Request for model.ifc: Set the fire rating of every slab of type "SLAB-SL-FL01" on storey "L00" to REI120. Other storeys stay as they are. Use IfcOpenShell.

First a look at what the model holds.

```python
import ifcopenshell
import ifcopenshell.util.element

model = ifcopenshell.open("model.ifc")
print(model.schema)
storey = next(s for s in model.by_type("IfcBuildingStorey") if s.Name == "L00")
slabs = [e for e in ifcopenshell.util.element.get_decomposition(storey) if e.is_a("IfcSlab")]
seen = {}
for e in slabs:
    element_type = ifcopenshell.util.element.get_type(e)
    key = (element_type.Name if element_type != e and element_type else None, ifcopenshell.util.element.get_pset(e, "Pset_SlabCommon", "FireRating"))
    seen[key] = seen.get(key, 0) + 1
for (name, value), count in sorted(seen.items(), key=str):
    print(count, "x", name, "|", value)
```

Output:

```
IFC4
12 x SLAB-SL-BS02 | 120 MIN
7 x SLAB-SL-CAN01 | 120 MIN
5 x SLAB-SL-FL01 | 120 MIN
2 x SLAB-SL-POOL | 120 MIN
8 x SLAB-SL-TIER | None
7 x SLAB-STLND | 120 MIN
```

```python
import ifcopenshell
import ifcopenshell.api.pset
import ifcopenshell.util.element

model = ifcopenshell.open("model.ifc")

storey = next(s for s in model.by_type("IfcBuildingStorey") if s.Name == "L00")
slabs = [e for e in ifcopenshell.util.element.get_decomposition(storey) if e.is_a("IfcSlab")]

count = 0
for e in slabs:
    element_type = ifcopenshell.util.element.get_type(e)
    if element_type in (None, e) or element_type.Name != "SLAB-SL-FL01":
        continue
    # add_pset returns the element's existing set when there is one.
    pset = ifcopenshell.api.pset.add_pset(model, product=e, name="Pset_SlabCommon")
    ifcopenshell.api.pset.edit_pset(model, pset=pset, properties={"FireRating": "REI120"})
    count += 1

print(count, "slabs updated")

model.write("model_v2.ifc")
```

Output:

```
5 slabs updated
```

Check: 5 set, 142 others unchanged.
